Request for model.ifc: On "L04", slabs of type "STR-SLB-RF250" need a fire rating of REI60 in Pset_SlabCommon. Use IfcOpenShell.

First a look at what the model holds.

```python
import ifcopenshell
import ifcopenshell.util.element

model = ifcopenshell.open("model.ifc")
print(model.schema)
storey = next(s for s in model.by_type("IfcBuildingStorey") if s.Name == "L04")
slabs = [e for e in ifcopenshell.util.element.get_decomposition(storey) if e.is_a("IfcSlab")]
seen = {}
for e in slabs:
    element_type = ifcopenshell.util.element.get_type(e)
    key = (element_type.Name if element_type != e and element_type else None, ifcopenshell.util.element.get_pset(e, "Pset_SlabCommon", "FireRating"))
    seen[key] = seen.get(key, 0) + 1
for (name, value), count in sorted(seen.items(), key=str):
    print(count, "x", name, "|", value)
```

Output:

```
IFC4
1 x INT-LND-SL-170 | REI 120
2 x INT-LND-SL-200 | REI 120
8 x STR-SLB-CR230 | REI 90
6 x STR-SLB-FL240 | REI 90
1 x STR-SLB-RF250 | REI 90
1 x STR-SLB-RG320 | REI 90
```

```python
import ifcopenshell
import ifcopenshell.api.pset
import ifcopenshell.util.element

model = ifcopenshell.open("model.ifc")

storey = next(s for s in model.by_type("IfcBuildingStorey") if s.Name == "L04")
slabs = [e for e in ifcopenshell.util.element.get_decomposition(storey) if e.is_a("IfcSlab")]

count = 0
for e in slabs:
    element_type = ifcopenshell.util.element.get_type(e)
    if element_type in (None, e) or element_type.Name != "STR-SLB-RF250":
        continue
    # add_pset returns the element's existing set when there is one.
    pset = ifcopenshell.api.pset.add_pset(model, product=e, name="Pset_SlabCommon")
    ifcopenshell.api.pset.edit_pset(model, pset=pset, properties={"FireRating": "REI60"})
    count += 1

print(count, "slabs updated")

model.write("model_updated.ifc")
```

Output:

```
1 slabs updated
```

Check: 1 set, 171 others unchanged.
